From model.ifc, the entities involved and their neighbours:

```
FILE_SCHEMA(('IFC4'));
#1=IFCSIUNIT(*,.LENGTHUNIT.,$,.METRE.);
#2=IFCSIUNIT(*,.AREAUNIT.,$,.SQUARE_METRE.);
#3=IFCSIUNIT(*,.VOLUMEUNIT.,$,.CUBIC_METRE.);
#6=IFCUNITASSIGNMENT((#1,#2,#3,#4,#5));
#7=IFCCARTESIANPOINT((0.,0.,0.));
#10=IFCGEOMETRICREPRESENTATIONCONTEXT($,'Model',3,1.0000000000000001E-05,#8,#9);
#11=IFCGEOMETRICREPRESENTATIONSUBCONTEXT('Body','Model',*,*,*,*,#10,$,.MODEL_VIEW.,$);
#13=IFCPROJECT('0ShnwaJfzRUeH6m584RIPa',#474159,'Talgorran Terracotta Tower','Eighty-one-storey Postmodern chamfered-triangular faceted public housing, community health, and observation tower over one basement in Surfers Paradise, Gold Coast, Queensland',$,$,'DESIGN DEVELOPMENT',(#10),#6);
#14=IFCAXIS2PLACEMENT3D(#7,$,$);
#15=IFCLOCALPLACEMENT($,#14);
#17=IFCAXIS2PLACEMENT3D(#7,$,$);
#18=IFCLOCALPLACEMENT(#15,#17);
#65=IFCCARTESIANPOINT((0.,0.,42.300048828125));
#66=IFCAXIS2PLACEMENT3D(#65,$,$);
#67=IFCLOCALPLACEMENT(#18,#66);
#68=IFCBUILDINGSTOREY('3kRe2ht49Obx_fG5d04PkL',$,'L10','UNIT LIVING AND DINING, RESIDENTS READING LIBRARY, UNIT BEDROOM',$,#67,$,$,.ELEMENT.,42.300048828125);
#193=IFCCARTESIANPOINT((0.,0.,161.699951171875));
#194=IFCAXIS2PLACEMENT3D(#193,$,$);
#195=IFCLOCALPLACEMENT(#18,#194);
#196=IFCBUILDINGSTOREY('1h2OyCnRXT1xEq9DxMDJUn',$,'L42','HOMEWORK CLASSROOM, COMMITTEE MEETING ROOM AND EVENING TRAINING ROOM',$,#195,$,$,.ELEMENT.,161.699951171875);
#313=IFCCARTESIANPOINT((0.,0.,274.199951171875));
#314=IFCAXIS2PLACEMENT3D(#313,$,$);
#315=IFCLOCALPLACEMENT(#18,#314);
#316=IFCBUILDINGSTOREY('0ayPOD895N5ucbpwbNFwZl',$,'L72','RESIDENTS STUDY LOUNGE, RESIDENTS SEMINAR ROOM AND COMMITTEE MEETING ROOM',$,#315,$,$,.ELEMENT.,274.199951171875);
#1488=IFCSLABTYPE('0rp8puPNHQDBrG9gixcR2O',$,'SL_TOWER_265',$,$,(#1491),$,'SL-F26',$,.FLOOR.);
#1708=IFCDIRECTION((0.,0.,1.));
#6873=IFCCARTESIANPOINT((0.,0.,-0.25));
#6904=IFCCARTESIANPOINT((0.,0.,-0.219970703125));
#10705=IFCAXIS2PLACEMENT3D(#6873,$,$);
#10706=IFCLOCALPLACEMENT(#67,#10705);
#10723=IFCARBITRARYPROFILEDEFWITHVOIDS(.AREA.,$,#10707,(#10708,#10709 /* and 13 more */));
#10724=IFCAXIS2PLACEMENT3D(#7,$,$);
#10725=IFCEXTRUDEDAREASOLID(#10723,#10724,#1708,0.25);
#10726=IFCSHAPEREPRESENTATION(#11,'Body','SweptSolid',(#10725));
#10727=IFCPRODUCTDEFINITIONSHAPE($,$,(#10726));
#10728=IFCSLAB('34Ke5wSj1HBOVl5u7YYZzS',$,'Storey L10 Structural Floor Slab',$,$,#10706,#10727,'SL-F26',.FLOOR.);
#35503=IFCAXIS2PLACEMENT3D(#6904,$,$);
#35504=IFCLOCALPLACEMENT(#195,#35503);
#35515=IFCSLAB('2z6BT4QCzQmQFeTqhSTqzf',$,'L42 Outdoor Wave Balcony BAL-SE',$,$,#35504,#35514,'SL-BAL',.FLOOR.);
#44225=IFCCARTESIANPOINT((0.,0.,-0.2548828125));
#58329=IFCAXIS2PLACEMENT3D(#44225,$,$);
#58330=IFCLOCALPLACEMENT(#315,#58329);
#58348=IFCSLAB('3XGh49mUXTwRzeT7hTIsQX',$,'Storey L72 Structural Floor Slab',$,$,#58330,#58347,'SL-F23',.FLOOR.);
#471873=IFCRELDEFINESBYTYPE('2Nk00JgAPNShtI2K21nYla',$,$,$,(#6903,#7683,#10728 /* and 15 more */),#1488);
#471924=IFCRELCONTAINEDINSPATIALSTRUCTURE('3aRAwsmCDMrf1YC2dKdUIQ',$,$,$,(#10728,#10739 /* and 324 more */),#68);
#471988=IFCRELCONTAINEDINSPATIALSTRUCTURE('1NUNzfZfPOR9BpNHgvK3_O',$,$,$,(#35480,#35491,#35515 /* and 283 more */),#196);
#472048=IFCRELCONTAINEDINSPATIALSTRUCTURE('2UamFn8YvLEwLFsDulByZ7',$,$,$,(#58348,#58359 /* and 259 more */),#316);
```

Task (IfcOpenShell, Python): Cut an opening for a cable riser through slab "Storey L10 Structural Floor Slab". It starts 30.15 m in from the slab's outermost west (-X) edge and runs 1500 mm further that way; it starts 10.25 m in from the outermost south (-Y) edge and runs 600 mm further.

```python
import numpy as np
import ifcopenshell
import ifcopenshell.api.feature
import ifcopenshell.api.geometry
import ifcopenshell.api.root
import ifcopenshell.geom
import ifcopenshell.util.placement
import ifcopenshell.util.representation
import ifcopenshell.util.shape
import ifcopenshell.util.unit

model = ifcopenshell.open("model.ifc")
unit_scale = ifcopenshell.util.unit.calculate_unit_scale(model)
settings = ifcopenshell.geom.settings()


def volume(element):
    """Net volume in cubic metres, openings subtracted."""
    shape = ifcopenshell.geom.create_shape(settings, element)
    return ifcopenshell.util.shape.get_volume(shape.geometry)


slab = model.by_guid("34Ke5wSj1HBOVl5u7YYZzS")
before = volume(slab)

# Extent in the slab's own axes, in metres. The edges named are its -X and -Y sides.
slab_shape = ifcopenshell.geom.create_shape(settings, slab)
vertices = ifcopenshell.util.shape.get_vertices(slab_shape.geometry)
x_min, y_min, bottom = vertices.min(axis=0)
top = vertices[:, 2].max()

opening = ifcopenshell.api.root.create_entity(model, ifc_class="IfcOpeningElement", name="Cable riser opening", predefined_type="OPENING")
context = ifcopenshell.util.representation.get_context(model, "Model", "Body", "MODEL_VIEW")
width, depth = 1.5, 0.6
outline = [(0.0, 0.0), (width, 0.0), (width, depth), (0.0, depth), (0.0, 0.0)]
# Overshoot both faces by 50 mm so the cut is clean.
shape = ifcopenshell.api.geometry.add_slab_representation(
    model, context=context, depth=top - bottom + 0.1, polyline=outline
)
ifcopenshell.api.geometry.assign_representation(model, product=opening, representation=shape)

matrix = ifcopenshell.util.placement.get_local_placement(slab.ObjectPlacement)
matrix[:, 3] = matrix @ np.append(np.array([x_min + 30.15, y_min + 10.25, bottom - 0.05]) / unit_scale, 1.0)
ifcopenshell.api.geometry.edit_object_placement(model, product=opening, matrix=matrix, is_si=False)
ifcopenshell.api.feature.add_feature(model, feature=opening, element=slab)

after = volume(slab)

print(f"slab volume {before:.3f} -> {after:.3f} m3")

model.write("model_updated.ifc")
```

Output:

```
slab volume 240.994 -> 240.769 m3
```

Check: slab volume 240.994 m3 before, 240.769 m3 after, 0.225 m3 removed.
